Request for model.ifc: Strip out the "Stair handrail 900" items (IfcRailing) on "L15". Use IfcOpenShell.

First a look at what the model holds.

```python
import ifcopenshell
import ifcopenshell.util.element

model = ifcopenshell.open("model.ifc")
print(model.schema)
storey = next(s for s in model.by_type("IfcBuildingStorey") if s.Name == "L15")
railings = [e for e in ifcopenshell.util.element.get_decomposition(storey) if e.is_a("IfcRailing")]
seen = {}
for e in railings:
    element_type = ifcopenshell.util.element.get_type(e)
    name = element_type.Name if element_type not in (None, e) else None
    seen[name] = seen.get(name, 0) + 1
for name, count in sorted(seen.items(), key=str):
    print(count, "x", name)
```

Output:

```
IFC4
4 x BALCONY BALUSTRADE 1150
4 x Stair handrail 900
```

```python
import ifcopenshell
import ifcopenshell.api.root
import ifcopenshell.util.element

model = ifcopenshell.open("model.ifc")

storey = next(s for s in model.by_type("IfcBuildingStorey") if s.Name == "L15")
railings = [e for e in ifcopenshell.util.element.get_decomposition(storey) if e.is_a("IfcRailing")]
targets = [e for e in railings if (t := ifcopenshell.util.element.get_type(e)) not in (None, e) and t.Name == "Stair handrail 900"]

for e in targets:
    ifcopenshell.api.root.remove_product(model, product=e)
print(len(targets), "removed")

model.write("model_v2.ifc")
```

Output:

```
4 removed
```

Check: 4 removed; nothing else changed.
